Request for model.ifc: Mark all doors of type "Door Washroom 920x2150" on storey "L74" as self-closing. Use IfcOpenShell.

First a look at what the model holds.

```python
import ifcopenshell
import ifcopenshell.util.element

model = ifcopenshell.open("model.ifc")
print(model.schema)
storey = next(s for s in model.by_type("IfcBuildingStorey") if s.Name == "L74")
doors = [e for e in ifcopenshell.util.element.get_decomposition(storey) if e.is_a("IfcDoor")]
seen = {}
for e in doors:
    element_type = ifcopenshell.util.element.get_type(e)
    key = (element_type.Name if element_type != e and element_type else None, ifcopenshell.util.element.get_pset(e, "Pset_DoorCommon", "SelfClosing"))
    seen[key] = seen.get(key, 0) + 1
for (name, value), count in sorted(seen.items(), key=str):
    print(count, "x", name, "|", value)
```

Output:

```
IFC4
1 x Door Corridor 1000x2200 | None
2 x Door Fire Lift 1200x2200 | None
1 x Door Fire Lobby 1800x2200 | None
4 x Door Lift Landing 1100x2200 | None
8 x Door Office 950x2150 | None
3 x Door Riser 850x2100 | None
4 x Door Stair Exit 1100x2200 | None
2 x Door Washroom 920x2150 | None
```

```python
import ifcopenshell
import ifcopenshell.api.pset
import ifcopenshell.util.element

model = ifcopenshell.open("model.ifc")

storey = next(s for s in model.by_type("IfcBuildingStorey") if s.Name == "L74")
doors = [e for e in ifcopenshell.util.element.get_decomposition(storey) if e.is_a("IfcDoor")]

count = 0
for e in doors:
    element_type = ifcopenshell.util.element.get_type(e)
    if element_type in (None, e) or element_type.Name != "Door Washroom 920x2150":
        continue
    found = ifcopenshell.util.element.get_pset(e, "Pset_DoorCommon", should_inherit=False)
    if found:
        pset = model.by_id(found["id"])
        if len(ifcopenshell.util.element.get_elements_by_pset(pset)) > 1:
            pset = ifcopenshell.api.pset.unshare_pset(model, products=[e], pset=pset)[0]
    else:
        pset = ifcopenshell.api.pset.add_pset(model, product=e, name="Pset_DoorCommon")
    ifcopenshell.api.pset.edit_pset(model, pset=pset, properties={"SelfClosing": True})
    count += 1

print(count, "doors updated")

model.write("model_edited.ifc")
```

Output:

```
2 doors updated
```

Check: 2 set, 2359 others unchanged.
